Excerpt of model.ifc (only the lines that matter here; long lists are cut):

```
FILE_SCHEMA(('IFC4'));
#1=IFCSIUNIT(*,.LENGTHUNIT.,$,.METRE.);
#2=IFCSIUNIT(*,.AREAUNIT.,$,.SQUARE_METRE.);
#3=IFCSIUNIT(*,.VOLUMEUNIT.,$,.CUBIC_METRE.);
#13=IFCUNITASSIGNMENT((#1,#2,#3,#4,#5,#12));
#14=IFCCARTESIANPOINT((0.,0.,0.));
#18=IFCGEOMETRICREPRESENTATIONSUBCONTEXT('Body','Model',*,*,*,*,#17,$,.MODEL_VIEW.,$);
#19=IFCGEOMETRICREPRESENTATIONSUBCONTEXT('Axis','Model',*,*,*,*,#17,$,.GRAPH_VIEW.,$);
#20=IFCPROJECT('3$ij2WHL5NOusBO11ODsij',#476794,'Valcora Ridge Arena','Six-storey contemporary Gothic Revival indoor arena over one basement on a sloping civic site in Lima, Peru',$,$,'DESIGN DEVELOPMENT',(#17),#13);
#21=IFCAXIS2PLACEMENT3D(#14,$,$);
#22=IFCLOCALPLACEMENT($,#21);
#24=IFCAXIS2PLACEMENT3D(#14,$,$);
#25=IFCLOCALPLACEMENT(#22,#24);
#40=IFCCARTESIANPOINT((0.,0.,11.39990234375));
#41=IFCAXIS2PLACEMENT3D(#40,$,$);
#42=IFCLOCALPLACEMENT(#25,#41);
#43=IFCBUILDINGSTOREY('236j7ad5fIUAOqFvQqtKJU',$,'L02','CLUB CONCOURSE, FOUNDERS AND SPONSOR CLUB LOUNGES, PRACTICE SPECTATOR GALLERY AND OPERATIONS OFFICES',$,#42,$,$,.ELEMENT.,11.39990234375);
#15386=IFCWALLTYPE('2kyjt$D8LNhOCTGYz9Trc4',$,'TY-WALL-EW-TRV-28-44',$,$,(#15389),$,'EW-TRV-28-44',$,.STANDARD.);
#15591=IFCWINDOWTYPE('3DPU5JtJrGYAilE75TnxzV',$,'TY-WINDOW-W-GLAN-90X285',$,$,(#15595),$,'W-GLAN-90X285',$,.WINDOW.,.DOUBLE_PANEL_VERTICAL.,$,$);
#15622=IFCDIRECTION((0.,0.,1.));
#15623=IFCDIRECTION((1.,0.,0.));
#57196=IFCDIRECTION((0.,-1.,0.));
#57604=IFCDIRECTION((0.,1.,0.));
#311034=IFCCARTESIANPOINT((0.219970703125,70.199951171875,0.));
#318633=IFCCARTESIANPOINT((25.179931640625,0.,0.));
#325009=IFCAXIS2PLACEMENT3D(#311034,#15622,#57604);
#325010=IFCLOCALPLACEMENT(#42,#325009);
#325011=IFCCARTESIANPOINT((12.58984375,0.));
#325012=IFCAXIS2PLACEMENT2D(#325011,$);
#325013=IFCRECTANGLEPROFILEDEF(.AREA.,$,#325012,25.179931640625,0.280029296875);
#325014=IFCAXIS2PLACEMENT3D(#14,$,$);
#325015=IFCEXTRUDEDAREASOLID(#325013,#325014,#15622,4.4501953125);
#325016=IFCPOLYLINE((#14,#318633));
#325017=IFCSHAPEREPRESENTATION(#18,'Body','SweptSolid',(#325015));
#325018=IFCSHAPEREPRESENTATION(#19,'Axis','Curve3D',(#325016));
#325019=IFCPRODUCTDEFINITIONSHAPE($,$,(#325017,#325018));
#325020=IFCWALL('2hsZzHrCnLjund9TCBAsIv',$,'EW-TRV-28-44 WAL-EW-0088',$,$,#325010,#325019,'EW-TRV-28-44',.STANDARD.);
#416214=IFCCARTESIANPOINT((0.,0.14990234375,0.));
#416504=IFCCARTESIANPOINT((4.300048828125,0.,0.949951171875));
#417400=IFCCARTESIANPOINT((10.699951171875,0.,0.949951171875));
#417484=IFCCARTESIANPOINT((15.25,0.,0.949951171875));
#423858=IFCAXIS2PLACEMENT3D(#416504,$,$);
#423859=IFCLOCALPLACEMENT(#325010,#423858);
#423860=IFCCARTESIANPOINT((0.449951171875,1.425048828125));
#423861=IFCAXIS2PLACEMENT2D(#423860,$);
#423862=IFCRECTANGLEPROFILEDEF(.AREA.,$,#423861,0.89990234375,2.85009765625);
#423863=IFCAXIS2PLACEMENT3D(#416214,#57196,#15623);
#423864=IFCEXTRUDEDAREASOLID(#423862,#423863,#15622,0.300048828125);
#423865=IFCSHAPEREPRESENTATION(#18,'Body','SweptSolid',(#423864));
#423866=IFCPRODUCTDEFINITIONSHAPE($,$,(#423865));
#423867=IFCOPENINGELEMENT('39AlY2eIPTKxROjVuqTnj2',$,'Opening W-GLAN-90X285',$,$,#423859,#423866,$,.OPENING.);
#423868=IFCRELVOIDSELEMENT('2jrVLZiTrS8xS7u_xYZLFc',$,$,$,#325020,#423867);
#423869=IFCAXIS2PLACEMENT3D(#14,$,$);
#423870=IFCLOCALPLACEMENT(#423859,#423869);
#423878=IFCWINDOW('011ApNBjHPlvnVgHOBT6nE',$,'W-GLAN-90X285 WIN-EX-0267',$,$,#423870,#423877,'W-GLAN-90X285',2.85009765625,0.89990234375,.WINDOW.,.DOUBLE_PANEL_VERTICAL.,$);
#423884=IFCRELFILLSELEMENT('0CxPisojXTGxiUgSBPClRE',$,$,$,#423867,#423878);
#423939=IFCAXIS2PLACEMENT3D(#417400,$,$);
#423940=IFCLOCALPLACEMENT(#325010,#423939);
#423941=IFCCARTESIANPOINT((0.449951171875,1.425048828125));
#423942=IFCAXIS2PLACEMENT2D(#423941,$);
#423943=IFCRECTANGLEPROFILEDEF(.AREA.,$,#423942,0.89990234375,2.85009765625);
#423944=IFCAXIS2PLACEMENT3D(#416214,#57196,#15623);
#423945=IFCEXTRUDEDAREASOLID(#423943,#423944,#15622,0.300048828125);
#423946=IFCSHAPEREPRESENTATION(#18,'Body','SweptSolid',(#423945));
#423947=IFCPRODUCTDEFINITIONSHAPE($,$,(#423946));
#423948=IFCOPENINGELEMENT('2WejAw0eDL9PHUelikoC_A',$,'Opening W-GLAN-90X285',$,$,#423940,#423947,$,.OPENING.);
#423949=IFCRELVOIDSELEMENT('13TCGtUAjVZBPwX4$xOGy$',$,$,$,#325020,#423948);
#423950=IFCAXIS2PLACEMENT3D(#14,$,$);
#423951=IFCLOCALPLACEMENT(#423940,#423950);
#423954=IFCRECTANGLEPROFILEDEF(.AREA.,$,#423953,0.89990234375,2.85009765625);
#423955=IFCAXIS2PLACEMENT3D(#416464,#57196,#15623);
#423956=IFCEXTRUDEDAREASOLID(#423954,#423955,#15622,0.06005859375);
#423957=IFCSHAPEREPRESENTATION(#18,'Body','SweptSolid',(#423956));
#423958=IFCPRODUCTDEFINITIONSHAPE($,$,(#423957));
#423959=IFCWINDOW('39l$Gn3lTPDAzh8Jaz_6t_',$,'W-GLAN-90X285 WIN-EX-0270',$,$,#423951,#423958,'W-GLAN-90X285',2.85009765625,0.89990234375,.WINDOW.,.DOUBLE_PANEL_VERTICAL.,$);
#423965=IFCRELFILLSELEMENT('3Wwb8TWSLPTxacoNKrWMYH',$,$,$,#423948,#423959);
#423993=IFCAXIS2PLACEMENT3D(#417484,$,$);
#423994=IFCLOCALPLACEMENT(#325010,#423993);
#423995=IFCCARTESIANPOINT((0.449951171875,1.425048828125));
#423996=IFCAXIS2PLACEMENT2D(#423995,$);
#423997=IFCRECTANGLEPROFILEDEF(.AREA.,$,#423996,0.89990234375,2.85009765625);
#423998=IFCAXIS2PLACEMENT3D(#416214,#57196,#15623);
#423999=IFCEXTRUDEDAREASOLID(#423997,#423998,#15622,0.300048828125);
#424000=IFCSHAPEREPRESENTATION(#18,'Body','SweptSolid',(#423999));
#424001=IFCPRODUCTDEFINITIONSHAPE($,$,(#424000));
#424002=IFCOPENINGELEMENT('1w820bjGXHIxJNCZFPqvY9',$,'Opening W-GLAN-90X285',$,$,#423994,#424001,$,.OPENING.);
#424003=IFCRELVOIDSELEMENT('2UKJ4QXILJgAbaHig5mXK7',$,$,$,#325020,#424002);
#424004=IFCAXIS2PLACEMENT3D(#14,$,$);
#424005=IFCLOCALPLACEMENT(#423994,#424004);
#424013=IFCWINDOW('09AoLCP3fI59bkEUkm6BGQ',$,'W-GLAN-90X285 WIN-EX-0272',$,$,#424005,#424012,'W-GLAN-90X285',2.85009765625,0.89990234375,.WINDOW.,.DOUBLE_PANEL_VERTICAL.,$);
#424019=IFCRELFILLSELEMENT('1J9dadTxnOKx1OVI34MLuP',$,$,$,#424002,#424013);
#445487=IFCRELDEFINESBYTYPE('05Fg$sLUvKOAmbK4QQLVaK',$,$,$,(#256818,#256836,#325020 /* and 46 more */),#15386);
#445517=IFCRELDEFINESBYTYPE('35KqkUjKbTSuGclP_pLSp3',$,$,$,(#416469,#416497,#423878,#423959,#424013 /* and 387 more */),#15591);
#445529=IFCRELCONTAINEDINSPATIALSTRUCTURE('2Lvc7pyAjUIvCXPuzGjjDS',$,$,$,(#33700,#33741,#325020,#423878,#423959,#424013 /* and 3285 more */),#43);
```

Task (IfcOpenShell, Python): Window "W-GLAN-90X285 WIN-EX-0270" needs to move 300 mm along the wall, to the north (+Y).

```python
import ifcopenshell
import ifcopenshell.api.geometry
import ifcopenshell.util.placement
import ifcopenshell.util.unit

model = ifcopenshell.open("model.ifc")
unit_scale = ifcopenshell.util.unit.calculate_unit_scale(model)

window = model.by_id(423959)
opening = window.FillsVoids[0].RelatingOpeningElement
wall = opening.VoidsElements[0].RelatingBuildingElement

wall_matrix = ifcopenshell.util.placement.get_local_placement(wall.ObjectPlacement)
shift = wall_matrix[:3, 0] * 0.3 / unit_scale
before = ifcopenshell.util.placement.get_local_placement(window.ObjectPlacement)[:3, 3].copy()

# The window is placed relative to its opening, so it follows when the opening moves.
matrix = ifcopenshell.util.placement.get_local_placement(opening.ObjectPlacement)
matrix[:3, 3] += shift
ifcopenshell.api.geometry.edit_object_placement(
    model, product=opening, matrix=matrix, is_si=False, should_transform_children=True
)

after = ifcopenshell.util.placement.get_local_placement(window.ObjectPlacement)[:3, 3]
print("window moved by", (after - before).round(3) + 0.0)

model.write("model_edited.ifc")
```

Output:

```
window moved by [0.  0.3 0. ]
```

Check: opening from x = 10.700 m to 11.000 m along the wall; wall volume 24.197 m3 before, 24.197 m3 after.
